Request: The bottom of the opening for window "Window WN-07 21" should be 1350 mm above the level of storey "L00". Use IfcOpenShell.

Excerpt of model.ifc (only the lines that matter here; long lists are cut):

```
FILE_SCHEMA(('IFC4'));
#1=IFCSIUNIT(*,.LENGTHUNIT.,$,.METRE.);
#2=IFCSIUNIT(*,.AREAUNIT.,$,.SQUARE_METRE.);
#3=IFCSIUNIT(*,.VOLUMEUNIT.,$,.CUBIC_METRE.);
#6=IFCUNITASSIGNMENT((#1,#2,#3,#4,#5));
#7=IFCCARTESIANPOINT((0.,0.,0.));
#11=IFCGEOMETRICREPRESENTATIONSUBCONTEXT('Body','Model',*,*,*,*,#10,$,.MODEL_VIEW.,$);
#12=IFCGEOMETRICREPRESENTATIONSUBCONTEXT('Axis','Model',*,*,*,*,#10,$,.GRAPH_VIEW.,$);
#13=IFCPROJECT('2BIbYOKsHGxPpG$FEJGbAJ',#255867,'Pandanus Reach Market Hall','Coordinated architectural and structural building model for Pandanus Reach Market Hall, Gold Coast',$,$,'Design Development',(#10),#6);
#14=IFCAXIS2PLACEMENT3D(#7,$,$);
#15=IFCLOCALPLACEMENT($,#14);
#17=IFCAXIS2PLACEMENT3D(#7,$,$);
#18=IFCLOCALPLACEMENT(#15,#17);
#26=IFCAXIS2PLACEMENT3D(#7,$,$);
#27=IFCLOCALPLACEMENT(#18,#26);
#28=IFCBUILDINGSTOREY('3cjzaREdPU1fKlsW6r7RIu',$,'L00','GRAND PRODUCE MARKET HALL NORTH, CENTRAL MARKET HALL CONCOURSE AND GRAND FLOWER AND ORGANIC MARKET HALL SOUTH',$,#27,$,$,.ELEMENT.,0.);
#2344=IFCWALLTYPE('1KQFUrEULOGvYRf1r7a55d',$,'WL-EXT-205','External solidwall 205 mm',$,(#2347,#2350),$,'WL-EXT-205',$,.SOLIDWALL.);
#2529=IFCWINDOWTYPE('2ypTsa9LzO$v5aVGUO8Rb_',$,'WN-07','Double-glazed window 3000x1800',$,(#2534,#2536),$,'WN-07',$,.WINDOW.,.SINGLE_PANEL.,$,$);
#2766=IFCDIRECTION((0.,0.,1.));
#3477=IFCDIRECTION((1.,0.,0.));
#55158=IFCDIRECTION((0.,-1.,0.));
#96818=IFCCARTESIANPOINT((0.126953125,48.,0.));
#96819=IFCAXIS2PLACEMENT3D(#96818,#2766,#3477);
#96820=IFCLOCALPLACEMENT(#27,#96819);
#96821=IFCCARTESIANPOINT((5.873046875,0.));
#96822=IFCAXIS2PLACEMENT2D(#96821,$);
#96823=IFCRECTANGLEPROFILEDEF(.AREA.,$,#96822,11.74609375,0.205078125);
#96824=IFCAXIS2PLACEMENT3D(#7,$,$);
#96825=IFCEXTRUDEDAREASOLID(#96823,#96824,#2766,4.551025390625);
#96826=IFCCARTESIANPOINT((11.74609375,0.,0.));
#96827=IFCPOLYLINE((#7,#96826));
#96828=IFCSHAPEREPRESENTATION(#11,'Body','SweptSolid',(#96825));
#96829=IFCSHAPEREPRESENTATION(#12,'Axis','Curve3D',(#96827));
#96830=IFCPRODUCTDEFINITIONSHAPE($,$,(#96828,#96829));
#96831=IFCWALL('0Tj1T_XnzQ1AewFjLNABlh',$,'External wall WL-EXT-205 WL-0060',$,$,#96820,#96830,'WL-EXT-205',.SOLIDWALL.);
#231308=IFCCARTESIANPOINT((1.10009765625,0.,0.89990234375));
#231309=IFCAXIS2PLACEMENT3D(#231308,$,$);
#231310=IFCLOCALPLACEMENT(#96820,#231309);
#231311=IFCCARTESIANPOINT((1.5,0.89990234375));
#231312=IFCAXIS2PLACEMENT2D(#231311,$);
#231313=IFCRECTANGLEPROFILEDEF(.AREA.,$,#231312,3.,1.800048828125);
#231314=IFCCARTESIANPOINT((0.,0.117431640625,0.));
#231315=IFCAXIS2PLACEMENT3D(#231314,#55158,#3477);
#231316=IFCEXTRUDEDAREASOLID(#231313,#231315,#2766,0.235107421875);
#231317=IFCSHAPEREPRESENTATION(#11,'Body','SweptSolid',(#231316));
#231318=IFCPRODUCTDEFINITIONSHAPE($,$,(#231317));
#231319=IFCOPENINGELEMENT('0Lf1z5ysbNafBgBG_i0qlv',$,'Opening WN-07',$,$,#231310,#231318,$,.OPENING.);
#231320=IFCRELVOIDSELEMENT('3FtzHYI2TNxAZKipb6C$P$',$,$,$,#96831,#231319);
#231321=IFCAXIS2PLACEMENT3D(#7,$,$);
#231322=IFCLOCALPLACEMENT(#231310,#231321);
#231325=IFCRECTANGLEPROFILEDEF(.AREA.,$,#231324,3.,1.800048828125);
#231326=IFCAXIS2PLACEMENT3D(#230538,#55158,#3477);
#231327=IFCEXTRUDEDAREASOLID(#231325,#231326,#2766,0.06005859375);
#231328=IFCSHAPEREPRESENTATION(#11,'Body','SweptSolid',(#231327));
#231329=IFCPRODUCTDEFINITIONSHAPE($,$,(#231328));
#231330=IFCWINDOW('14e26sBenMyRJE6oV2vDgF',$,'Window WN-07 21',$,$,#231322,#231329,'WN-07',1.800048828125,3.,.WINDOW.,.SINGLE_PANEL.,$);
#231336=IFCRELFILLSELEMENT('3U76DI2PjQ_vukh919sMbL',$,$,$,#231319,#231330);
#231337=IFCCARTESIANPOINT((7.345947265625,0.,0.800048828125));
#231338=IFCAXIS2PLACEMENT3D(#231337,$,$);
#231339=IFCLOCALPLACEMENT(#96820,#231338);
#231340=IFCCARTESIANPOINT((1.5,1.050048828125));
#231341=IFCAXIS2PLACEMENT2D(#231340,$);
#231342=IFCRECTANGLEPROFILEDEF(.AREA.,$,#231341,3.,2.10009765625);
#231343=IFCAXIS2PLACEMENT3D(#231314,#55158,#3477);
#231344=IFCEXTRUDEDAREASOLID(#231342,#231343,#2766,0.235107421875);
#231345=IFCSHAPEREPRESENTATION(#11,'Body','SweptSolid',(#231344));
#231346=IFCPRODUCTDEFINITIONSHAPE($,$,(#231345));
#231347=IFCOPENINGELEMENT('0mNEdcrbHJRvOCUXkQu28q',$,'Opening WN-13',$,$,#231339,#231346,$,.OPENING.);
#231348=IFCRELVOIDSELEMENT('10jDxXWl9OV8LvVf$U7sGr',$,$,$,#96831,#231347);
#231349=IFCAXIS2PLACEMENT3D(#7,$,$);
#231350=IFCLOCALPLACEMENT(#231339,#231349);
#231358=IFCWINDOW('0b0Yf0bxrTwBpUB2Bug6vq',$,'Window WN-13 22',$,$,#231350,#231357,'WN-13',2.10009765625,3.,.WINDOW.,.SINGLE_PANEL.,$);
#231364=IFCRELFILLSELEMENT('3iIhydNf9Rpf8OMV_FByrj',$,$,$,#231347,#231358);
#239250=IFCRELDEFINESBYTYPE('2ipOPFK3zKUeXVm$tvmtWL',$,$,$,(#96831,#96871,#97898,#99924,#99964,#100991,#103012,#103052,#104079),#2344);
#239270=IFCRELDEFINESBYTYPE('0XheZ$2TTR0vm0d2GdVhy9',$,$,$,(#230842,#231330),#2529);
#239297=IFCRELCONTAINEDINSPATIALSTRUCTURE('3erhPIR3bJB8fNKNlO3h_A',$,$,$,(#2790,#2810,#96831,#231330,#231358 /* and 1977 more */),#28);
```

```python
import numpy as np
import ifcopenshell
import ifcopenshell.api.geometry
import ifcopenshell.geom
import ifcopenshell.util.element
import ifcopenshell.util.placement
import ifcopenshell.util.shape
import ifcopenshell.util.unit

model = ifcopenshell.open("model.ifc")
unit_scale = ifcopenshell.util.unit.calculate_unit_scale(model)

window = model.by_guid("14e26sBenMyRJE6oV2vDgF")
opening = window.FillsVoids[0].RelatingOpeningElement
storey = ifcopenshell.util.element.get_container(window, ifc_class="IfcBuildingStorey")
level = ifcopenshell.util.placement.get_local_placement(storey.ObjectPlacement)[2, 3]

# The opening's origin need not be at the sill, so measure its lowest point.
shape = ifcopenshell.geom.create_shape(ifcopenshell.geom.settings(), opening)
bottom = ifcopenshell.util.shape.get_shape_bottom_elevation(shape, shape.geometry) / unit_scale
dz = level + 1.35 / unit_scale - bottom

shift = np.array([0.0, 0.0, dz])
# The window is placed relative to its opening, so it follows when the opening moves.
matrix = ifcopenshell.util.placement.get_local_placement(opening.ObjectPlacement)
matrix[:3, 3] += shift
ifcopenshell.api.geometry.edit_object_placement(
    model, product=opening, matrix=matrix, is_si=False, should_transform_children=True
)

print(f"moved by {dz * unit_scale:+.3f} m")

model.write("model_v2.ifc")
```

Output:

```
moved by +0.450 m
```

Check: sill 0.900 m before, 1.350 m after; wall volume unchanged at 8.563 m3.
